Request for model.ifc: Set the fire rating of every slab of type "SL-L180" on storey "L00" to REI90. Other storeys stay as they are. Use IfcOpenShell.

First a look at what the model holds.

```python
import ifcopenshell
import ifcopenshell.util.element

model = ifcopenshell.open("model.ifc")
print(model.schema)
storey = next(s for s in model.by_type("IfcBuildingStorey") if s.Name == "L00")
slabs = [e for e in ifcopenshell.util.element.get_decomposition(storey) if e.is_a("IfcSlab")]
seen = {}
for e in slabs:
    element_type = ifcopenshell.util.element.get_type(e)
    key = (element_type.Name if element_type != e and element_type else None, ifcopenshell.util.element.get_pset(e, "Pset_SlabCommon", "FireRating"))
    seen[key] = seen.get(key, 0) + 1
for (name, value), count in sorted(seen.items(), key=str):
    print(count, "x", name, "|", value)
```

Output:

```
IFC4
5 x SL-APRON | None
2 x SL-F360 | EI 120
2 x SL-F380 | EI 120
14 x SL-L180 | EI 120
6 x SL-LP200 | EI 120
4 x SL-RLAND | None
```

```python
import ifcopenshell
import ifcopenshell.api.pset
import ifcopenshell.util.element

model = ifcopenshell.open("model.ifc")

storey = next(s for s in model.by_type("IfcBuildingStorey") if s.Name == "L00")
slabs = [e for e in ifcopenshell.util.element.get_decomposition(storey) if e.is_a("IfcSlab")]

count = 0
for e in slabs:
    element_type = ifcopenshell.util.element.get_type(e)
    if element_type in (None, e) or element_type.Name != "SL-L180":
        continue
    # add_pset returns the element's existing set when there is one.
    pset = ifcopenshell.api.pset.add_pset(model, product=e, name="Pset_SlabCommon")
    ifcopenshell.api.pset.edit_pset(model, pset=pset, properties={"FireRating": "REI90"})
    count += 1

print(count, "slabs updated")

model.write("model_edited.ifc")
```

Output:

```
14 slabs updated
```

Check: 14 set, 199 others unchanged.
